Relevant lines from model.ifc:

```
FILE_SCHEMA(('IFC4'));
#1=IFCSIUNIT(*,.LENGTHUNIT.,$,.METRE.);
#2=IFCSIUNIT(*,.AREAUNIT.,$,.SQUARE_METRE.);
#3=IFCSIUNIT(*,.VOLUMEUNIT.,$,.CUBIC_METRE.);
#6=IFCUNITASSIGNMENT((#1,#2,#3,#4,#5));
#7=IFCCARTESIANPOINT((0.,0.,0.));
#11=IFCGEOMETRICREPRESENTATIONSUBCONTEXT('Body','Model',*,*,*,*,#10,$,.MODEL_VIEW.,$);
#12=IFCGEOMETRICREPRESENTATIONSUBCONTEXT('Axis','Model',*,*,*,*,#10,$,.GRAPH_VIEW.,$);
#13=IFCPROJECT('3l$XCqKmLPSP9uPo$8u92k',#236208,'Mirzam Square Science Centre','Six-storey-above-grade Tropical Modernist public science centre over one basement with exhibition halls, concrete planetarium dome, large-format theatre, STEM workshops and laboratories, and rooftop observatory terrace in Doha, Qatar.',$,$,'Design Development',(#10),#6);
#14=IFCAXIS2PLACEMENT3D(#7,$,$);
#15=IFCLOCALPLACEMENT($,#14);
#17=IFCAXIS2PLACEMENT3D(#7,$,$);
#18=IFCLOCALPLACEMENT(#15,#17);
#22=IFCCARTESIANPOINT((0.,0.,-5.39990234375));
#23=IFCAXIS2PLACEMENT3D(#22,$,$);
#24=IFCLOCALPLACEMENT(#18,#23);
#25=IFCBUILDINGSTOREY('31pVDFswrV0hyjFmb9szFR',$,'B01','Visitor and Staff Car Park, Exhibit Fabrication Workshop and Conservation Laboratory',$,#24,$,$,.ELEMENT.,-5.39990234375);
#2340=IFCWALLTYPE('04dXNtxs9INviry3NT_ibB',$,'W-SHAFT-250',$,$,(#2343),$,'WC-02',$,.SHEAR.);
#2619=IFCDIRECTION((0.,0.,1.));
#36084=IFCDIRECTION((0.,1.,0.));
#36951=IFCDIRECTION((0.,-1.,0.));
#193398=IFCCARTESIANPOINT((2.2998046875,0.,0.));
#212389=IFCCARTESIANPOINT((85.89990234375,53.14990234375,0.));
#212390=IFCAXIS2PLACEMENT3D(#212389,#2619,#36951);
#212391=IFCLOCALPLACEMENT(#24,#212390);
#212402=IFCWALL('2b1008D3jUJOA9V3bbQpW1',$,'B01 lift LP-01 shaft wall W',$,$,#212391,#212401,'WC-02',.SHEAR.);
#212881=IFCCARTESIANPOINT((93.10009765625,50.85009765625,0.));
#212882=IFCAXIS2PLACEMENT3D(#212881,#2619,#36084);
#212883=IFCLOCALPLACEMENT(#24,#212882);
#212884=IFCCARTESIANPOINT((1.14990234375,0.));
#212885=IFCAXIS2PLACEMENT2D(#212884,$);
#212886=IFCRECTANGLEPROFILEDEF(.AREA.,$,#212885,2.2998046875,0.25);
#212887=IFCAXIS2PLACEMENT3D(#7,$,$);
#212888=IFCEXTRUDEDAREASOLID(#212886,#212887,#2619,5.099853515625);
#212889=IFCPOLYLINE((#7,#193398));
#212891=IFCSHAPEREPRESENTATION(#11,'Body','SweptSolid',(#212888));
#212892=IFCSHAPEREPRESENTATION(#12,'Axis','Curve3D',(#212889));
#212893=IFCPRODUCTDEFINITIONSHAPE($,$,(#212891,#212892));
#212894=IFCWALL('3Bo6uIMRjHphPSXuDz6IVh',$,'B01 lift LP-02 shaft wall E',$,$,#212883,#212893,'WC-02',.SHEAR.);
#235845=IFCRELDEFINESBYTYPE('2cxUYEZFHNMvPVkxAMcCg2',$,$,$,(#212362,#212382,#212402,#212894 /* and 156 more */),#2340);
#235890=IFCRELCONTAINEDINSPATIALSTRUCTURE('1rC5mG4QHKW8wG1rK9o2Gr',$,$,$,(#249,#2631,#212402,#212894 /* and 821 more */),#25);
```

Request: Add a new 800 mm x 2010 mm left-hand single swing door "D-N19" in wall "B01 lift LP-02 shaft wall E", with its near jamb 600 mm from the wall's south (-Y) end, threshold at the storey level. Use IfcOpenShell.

```python
import numpy as np
import ifcopenshell
import ifcopenshell.api.feature
import ifcopenshell.api.geometry
import ifcopenshell.api.root
import ifcopenshell.api.spatial
import ifcopenshell.geom
import ifcopenshell.util.element
import ifcopenshell.util.placement
import ifcopenshell.util.representation
import ifcopenshell.util.shape
import ifcopenshell.util.unit

model = ifcopenshell.open("model.ifc")
unit_scale = ifcopenshell.util.unit.calculate_unit_scale(model)
settings = ifcopenshell.geom.settings()


def volume(element):
    """Net volume in cubic metres, openings subtracted."""
    shape = ifcopenshell.geom.create_shape(settings, element)
    return ifcopenshell.util.shape.get_volume(shape.geometry)


wall = model.by_guid("3Bo6uIMRjHphPSXuDz6IVh")
storey = ifcopenshell.util.element.get_container(wall, ifc_class="IfcBuildingStorey")
context = ifcopenshell.util.representation.get_context(model, "Model", "Body", "MODEL_VIEW")
before = volume(wall)

width, height, from_end, sill = 0.8, 2.01, 0.6, 0.0  # metres

# The wall runs along its own X axis, and the end named is its -X end.
wall_shape = ifcopenshell.geom.create_shape(settings, wall)
x, y, z = ifcopenshell.util.shape.get_vertices(wall_shape.geometry).T
start = x.min() + from_end
face, thickness = float(y.min()), float(y.max() - y.min())
wall_matrix = ifcopenshell.util.placement.get_local_placement(wall.ObjectPlacement)
level = ifcopenshell.util.placement.get_local_placement(storey.ObjectPlacement)[2, 3]


def in_wall(x, y):
    """Placement at x, y metres in the wall's axes, at sill height."""
    matrix = wall_matrix.copy()
    matrix[:, 3] = wall_matrix @ np.array([x / unit_scale, y / unit_scale, 0.0, 1.0])
    matrix[2, 3] = level + sill / unit_scale
    return matrix


# Opening: a box that overshoots both wall faces by 50 mm.
opening = ifcopenshell.api.root.create_entity(model, ifc_class="IfcOpeningElement", predefined_type="OPENING")
box = ifcopenshell.api.geometry.add_wall_representation(
    model, context=context, length=width, height=height, thickness=thickness + 0.1
)
ifcopenshell.api.geometry.assign_representation(model, product=opening, representation=box)
ifcopenshell.api.geometry.edit_object_placement(model, product=opening, matrix=in_wall(start, face - 0.05), is_si=False)
ifcopenshell.api.feature.add_feature(model, feature=opening, element=wall)

door = ifcopenshell.api.root.create_entity(model, ifc_class="IfcDoor", name="D-N19", predefined_type="DOOR")
door.OverallWidth, door.OverallHeight = width / unit_scale, height / unit_scale
door.OperationType = "SINGLE_SWING_LEFT"
body = ifcopenshell.api.geometry.add_door_representation(
    model,
    context=context,
    overall_width=door.OverallWidth,
    overall_height=door.OverallHeight,
    operation_type="SINGLE_SWING_LEFT",
    lining_properties={"LiningDepth": thickness / unit_scale, "ThresholdDepth": thickness / unit_scale},
)
ifcopenshell.api.geometry.assign_representation(model, product=door, representation=body)
ifcopenshell.api.spatial.assign_container(model, products=[door], relating_structure=storey)
ifcopenshell.api.feature.add_filling(model, opening=opening, element=door)

# The lining spans the wall, so the door starts at the wall face.
ifcopenshell.api.geometry.edit_object_placement(model, product=door, matrix=in_wall(start, face), is_si=False)

after = volume(wall)

print(f"wall volume {before:.3f} -> {after:.3f} m3")

model.write("model_rev.ifc")
```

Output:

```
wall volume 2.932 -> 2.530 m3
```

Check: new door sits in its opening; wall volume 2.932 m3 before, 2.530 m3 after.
